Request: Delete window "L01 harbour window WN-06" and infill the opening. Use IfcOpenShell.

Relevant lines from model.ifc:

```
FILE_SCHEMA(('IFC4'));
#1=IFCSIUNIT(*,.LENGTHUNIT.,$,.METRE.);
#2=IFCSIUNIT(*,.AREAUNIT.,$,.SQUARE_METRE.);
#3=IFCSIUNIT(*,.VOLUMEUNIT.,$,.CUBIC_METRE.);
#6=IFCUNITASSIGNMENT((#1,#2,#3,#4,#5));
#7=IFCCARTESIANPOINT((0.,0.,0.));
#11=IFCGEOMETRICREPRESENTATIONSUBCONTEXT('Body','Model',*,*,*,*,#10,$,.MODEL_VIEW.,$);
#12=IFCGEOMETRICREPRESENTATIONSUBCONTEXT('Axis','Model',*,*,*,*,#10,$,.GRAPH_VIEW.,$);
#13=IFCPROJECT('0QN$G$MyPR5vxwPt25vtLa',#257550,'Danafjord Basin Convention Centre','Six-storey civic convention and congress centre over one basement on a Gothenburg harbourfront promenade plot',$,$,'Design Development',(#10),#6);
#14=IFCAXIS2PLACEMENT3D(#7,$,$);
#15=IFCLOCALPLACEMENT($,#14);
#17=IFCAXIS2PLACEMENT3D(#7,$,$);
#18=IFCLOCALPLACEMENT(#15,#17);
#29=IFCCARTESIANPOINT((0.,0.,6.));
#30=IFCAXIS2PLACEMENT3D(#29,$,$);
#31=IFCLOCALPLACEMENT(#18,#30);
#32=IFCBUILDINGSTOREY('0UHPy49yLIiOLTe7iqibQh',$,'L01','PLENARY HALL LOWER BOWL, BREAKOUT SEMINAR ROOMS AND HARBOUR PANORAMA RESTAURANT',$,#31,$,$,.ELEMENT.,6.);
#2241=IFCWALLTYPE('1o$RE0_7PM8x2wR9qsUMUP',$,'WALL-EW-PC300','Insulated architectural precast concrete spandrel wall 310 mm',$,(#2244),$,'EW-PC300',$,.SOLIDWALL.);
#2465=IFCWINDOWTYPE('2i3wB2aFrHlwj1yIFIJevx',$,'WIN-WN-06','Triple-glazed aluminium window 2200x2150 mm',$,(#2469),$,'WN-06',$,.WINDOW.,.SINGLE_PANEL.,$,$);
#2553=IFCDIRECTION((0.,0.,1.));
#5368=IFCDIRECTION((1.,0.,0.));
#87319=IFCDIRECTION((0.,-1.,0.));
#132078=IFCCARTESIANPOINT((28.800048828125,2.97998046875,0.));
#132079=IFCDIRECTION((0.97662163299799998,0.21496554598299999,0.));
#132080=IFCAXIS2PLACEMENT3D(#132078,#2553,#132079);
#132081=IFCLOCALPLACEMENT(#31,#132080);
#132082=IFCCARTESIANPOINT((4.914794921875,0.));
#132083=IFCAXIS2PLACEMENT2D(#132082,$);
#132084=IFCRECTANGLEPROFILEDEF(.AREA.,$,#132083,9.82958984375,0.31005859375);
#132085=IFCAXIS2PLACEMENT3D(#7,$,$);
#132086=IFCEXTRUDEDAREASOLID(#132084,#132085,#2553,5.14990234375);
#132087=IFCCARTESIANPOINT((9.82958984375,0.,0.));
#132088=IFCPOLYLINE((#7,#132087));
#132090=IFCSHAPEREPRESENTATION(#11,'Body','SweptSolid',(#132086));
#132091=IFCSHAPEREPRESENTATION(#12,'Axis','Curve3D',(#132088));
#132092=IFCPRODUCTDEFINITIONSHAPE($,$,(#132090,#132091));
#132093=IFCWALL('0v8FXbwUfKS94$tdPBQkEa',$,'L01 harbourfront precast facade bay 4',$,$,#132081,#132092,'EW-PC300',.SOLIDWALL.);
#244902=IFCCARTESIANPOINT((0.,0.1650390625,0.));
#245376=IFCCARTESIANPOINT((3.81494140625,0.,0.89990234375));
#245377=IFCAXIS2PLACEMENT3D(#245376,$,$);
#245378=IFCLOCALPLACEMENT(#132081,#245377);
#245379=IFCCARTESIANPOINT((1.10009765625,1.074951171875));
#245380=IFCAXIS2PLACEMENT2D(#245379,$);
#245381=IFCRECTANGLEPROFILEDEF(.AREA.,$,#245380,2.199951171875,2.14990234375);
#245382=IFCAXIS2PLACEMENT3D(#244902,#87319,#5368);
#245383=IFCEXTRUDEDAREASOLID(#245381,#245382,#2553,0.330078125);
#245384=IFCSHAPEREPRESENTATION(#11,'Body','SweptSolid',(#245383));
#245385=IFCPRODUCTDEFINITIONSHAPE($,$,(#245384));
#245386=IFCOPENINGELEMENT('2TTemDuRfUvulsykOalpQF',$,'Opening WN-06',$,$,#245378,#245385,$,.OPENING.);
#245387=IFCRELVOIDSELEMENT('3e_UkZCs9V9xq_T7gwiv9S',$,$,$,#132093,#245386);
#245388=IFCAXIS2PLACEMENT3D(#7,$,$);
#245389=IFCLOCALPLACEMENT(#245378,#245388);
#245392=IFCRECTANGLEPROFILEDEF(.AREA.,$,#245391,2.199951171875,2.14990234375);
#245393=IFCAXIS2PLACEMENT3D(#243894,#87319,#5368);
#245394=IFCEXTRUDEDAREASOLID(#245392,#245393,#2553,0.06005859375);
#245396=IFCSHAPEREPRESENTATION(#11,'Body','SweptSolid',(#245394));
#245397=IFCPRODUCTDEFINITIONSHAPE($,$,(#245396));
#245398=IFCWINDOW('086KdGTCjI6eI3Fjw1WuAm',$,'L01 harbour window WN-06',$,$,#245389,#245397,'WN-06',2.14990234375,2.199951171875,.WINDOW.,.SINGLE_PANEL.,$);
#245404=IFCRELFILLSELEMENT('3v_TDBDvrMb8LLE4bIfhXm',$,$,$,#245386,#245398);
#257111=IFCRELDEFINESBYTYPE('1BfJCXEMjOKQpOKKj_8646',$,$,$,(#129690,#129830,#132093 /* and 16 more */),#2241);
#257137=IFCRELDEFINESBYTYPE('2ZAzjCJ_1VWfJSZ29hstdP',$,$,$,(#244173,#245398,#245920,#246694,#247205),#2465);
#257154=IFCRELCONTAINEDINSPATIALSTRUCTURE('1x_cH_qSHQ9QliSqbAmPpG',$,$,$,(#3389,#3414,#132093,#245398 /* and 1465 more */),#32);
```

```python
import ifcopenshell
import ifcopenshell.api.feature
import ifcopenshell.api.root
import ifcopenshell.geom
import ifcopenshell.util.shape

model = ifcopenshell.open("model.ifc")
settings = ifcopenshell.geom.settings()


def volume(element):
    """Net volume in cubic metres, openings subtracted."""
    shape = ifcopenshell.geom.create_shape(settings, element)
    return ifcopenshell.util.shape.get_volume(shape.geometry)


window = model.by_id(245398)
opening = window.FillsVoids[0].RelatingOpeningElement
wall = opening.VoidsElements[0].RelatingBuildingElement
before = volume(wall)

ifcopenshell.api.root.remove_product(model, product=window)
ifcopenshell.api.feature.remove_feature(model, feature=opening)

after = volume(wall)

print(f"wall volume {before:.3f} -> {after:.3f} m3")

model.write("model_edited.ifc")
```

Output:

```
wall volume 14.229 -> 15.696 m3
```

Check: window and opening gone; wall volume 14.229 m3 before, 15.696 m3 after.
